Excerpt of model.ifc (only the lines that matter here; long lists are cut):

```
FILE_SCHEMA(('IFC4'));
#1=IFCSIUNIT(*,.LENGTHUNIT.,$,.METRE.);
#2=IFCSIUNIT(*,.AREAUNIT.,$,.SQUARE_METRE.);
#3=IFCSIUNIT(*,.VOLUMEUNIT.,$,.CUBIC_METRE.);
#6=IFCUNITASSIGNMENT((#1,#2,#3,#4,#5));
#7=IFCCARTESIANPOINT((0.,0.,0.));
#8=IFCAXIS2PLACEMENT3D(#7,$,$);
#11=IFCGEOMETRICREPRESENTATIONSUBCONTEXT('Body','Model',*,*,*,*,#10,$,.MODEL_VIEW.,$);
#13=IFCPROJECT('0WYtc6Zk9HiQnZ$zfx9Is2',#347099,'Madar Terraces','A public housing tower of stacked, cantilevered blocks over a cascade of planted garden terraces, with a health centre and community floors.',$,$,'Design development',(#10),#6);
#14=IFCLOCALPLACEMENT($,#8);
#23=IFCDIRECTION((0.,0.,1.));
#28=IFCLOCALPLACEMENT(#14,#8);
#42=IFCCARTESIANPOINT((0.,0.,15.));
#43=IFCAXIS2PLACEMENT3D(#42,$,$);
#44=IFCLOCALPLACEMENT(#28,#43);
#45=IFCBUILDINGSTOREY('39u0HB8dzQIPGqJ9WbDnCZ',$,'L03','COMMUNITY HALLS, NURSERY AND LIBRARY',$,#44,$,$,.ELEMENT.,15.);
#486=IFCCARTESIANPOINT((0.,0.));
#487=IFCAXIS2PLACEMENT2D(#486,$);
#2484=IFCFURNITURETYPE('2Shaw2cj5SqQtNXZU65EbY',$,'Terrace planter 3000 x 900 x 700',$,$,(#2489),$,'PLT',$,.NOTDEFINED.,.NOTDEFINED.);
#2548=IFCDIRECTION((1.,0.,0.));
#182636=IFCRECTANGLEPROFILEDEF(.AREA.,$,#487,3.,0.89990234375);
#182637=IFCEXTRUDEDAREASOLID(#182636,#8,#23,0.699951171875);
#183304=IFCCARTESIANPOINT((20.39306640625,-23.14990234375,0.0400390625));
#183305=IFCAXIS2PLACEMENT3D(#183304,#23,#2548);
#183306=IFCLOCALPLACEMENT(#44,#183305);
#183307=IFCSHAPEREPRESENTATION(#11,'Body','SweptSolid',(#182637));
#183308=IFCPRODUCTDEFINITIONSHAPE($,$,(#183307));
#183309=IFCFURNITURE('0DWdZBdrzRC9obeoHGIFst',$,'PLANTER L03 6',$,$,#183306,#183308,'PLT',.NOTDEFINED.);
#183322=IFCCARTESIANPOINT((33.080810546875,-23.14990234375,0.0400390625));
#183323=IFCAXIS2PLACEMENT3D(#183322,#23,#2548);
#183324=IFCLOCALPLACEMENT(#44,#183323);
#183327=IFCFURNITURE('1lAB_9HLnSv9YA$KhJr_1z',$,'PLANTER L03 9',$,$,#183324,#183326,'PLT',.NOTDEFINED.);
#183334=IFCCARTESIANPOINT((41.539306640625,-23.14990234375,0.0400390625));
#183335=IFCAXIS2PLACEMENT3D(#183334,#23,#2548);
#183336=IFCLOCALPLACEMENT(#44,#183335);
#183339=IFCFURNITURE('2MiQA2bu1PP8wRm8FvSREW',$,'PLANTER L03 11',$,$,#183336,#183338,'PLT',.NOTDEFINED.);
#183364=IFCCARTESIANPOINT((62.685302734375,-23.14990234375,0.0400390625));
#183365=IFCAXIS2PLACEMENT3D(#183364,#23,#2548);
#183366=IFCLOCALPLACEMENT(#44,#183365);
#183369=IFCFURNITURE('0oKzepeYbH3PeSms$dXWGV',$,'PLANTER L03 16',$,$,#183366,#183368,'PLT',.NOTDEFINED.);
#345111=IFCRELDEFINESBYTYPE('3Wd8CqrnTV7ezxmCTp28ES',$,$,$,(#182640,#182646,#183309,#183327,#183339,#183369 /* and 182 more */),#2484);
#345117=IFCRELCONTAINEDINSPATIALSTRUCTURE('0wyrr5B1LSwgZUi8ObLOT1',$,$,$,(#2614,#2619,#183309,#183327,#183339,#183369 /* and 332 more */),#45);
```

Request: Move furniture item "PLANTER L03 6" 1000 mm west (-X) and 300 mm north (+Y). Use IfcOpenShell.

```python
import ifcopenshell
import ifcopenshell.api.geometry
import ifcopenshell.util.placement
import ifcopenshell.util.unit

model = ifcopenshell.open("model.ifc")
unit_scale = ifcopenshell.util.unit.calculate_unit_scale(model)

item = model.by_id(183309)
matrix = ifcopenshell.util.placement.get_local_placement(item.ObjectPlacement)
matrix[0, 3] -= 1 / unit_scale
matrix[1, 3] += 0.3 / unit_scale
ifcopenshell.api.geometry.edit_object_placement(model, product=item, matrix=matrix, is_si=False)

print(ifcopenshell.util.placement.get_local_placement(item.ObjectPlacement).round(3) + 0.0)

model.write("model_rev.ifc")
```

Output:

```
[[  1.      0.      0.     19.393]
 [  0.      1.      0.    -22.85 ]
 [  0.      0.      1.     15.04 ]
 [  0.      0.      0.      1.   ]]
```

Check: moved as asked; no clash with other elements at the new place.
